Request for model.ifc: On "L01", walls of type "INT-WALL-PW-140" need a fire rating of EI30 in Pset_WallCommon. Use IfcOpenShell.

First a look at what the model holds.

```python
import ifcopenshell
import ifcopenshell.util.element

model = ifcopenshell.open("model.ifc")
print(model.schema)
storey = next(s for s in model.by_type("IfcBuildingStorey") if s.Name == "L01")
walls = [e for e in ifcopenshell.util.element.get_decomposition(storey) if e.is_a("IfcWall")]
seen = {}
for e in walls:
    element_type = ifcopenshell.util.element.get_type(e)
    key = (element_type.Name if element_type != e and element_type else None, ifcopenshell.util.element.get_pset(e, "Pset_WallCommon", "FireRating"))
    seen[key] = seen.get(key, 0) + 1
for (name, value), count in sorted(seen.items(), key=str):
    print(count, "x", name, "|", value)
```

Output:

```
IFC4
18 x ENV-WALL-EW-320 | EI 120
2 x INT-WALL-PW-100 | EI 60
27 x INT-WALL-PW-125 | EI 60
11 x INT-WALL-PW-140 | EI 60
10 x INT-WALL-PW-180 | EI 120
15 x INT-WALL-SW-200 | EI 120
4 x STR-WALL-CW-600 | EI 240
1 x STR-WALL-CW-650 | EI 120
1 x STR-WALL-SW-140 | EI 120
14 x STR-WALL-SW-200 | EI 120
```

```python
import ifcopenshell
import ifcopenshell.api.pset
import ifcopenshell.util.element

model = ifcopenshell.open("model.ifc")

storey = next(s for s in model.by_type("IfcBuildingStorey") if s.Name == "L01")
walls = [e for e in ifcopenshell.util.element.get_decomposition(storey) if e.is_a("IfcWall")]

count = 0
for e in walls:
    element_type = ifcopenshell.util.element.get_type(e)
    if element_type in (None, e) or element_type.Name != "INT-WALL-PW-140":
        continue
    found = ifcopenshell.util.element.get_pset(e, "Pset_WallCommon", should_inherit=False)
    if found:
        pset = model.by_id(found["id"])
        if len(ifcopenshell.util.element.get_elements_by_pset(pset)) > 1:
            pset = ifcopenshell.api.pset.unshare_pset(model, products=[e], pset=pset)[0]
    else:
        pset = ifcopenshell.api.pset.add_pset(model, product=e, name="Pset_WallCommon")
    ifcopenshell.api.pset.edit_pset(model, pset=pset, properties={"FireRating": "EI30"})
    count += 1

print(count, "walls updated")

model.write("model_rev.ifc")
```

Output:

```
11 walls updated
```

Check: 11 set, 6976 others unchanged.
